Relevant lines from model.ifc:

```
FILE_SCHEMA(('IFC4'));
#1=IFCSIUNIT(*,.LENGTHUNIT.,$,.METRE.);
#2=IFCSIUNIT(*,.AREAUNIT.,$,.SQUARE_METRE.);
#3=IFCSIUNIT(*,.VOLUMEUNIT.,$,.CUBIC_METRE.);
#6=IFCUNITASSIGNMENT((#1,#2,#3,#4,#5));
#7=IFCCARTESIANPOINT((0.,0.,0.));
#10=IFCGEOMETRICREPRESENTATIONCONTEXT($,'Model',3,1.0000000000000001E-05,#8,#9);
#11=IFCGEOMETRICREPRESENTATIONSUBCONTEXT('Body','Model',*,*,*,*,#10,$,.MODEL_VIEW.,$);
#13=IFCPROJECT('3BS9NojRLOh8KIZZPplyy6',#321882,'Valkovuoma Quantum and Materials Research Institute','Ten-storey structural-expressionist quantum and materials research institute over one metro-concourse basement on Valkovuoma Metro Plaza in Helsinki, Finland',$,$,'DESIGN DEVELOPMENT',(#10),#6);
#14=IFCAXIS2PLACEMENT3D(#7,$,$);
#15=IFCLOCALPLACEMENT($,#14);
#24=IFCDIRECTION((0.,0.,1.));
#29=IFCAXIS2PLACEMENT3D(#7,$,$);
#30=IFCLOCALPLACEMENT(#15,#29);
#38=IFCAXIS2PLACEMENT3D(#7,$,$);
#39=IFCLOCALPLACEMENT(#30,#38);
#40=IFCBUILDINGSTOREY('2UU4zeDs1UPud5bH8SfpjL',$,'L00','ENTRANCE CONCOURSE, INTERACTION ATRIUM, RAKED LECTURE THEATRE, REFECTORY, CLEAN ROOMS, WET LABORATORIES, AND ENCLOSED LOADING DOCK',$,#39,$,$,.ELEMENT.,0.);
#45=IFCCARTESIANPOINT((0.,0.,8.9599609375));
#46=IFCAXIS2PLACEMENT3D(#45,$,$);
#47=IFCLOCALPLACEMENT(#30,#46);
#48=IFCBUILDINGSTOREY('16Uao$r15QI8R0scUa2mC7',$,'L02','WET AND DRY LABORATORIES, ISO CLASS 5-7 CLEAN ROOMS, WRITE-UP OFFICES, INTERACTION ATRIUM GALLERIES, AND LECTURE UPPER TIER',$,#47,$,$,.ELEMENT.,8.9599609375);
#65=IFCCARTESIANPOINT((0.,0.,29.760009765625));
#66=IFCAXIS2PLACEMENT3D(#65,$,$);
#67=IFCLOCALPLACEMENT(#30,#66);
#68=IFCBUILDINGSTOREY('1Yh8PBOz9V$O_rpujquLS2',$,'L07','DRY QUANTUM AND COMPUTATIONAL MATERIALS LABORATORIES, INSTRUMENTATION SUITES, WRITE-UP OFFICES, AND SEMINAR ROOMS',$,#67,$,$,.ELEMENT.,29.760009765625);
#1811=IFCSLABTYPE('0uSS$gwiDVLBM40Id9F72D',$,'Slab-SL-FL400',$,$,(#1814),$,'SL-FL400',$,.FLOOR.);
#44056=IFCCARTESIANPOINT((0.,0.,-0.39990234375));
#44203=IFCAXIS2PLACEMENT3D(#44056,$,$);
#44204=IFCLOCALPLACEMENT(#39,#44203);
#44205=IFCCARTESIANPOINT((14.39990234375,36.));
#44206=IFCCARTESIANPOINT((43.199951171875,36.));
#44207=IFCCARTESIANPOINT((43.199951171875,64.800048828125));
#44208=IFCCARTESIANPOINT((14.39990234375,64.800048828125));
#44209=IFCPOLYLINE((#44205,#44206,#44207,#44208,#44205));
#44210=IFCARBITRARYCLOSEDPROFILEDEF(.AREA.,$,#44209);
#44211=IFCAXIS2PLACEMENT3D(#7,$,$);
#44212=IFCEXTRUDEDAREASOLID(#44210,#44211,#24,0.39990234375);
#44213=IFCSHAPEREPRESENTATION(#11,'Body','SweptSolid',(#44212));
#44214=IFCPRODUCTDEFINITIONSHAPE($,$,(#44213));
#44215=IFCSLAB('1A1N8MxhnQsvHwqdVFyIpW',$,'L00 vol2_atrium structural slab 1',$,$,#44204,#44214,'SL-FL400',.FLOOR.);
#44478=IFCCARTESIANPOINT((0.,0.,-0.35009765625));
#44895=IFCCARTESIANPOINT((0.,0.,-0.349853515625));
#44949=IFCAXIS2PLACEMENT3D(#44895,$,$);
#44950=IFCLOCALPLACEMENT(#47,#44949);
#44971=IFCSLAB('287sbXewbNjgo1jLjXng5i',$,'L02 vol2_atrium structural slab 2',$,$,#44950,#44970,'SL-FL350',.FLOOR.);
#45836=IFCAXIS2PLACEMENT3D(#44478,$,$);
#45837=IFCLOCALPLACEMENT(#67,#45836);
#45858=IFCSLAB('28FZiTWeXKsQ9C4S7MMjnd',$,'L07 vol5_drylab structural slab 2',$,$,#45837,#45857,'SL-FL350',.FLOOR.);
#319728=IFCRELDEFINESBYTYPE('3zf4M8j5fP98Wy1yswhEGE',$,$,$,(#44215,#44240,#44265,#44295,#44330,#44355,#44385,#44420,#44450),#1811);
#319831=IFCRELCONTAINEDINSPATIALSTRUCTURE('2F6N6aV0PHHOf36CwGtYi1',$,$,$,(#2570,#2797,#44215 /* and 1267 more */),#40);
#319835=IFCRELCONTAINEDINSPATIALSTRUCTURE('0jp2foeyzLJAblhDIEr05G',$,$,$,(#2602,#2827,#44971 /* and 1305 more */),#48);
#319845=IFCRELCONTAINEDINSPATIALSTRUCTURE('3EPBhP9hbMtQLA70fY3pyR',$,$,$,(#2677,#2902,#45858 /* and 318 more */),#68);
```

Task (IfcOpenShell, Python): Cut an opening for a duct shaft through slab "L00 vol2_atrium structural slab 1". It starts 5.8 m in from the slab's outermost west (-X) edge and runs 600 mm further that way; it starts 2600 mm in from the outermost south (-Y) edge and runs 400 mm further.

```python
import numpy as np
import ifcopenshell
import ifcopenshell.api.feature
import ifcopenshell.api.geometry
import ifcopenshell.api.root
import ifcopenshell.geom
import ifcopenshell.util.placement
import ifcopenshell.util.representation
import ifcopenshell.util.shape
import ifcopenshell.util.unit

model = ifcopenshell.open("model.ifc")
unit_scale = ifcopenshell.util.unit.calculate_unit_scale(model)
settings = ifcopenshell.geom.settings()


def volume(element):
    """Net volume in cubic metres, openings subtracted."""
    shape = ifcopenshell.geom.create_shape(settings, element)
    return ifcopenshell.util.shape.get_volume(shape.geometry)


slab = model.by_guid("1A1N8MxhnQsvHwqdVFyIpW")
before = volume(slab)

# Extent in the slab's own axes, in metres. The edges named are its -X and -Y sides.
slab_shape = ifcopenshell.geom.create_shape(settings, slab)
vertices = ifcopenshell.util.shape.get_vertices(slab_shape.geometry)
x_min, y_min, bottom = vertices.min(axis=0)
top = vertices[:, 2].max()

opening = ifcopenshell.api.root.create_entity(model, ifc_class="IfcOpeningElement", name="Duct shaft opening", predefined_type="OPENING")
context = ifcopenshell.util.representation.get_context(model, "Model", "Body", "MODEL_VIEW")
width, depth = 0.6, 0.4
outline = [(0.0, 0.0), (width, 0.0), (width, depth), (0.0, depth), (0.0, 0.0)]
# Overshoot both faces by 50 mm so the cut is clean.
shape = ifcopenshell.api.geometry.add_slab_representation(
    model, context=context, depth=top - bottom + 0.1, polyline=outline
)
ifcopenshell.api.geometry.assign_representation(model, product=opening, representation=shape)

matrix = ifcopenshell.util.placement.get_local_placement(slab.ObjectPlacement)
matrix[:, 3] = matrix @ np.append(np.array([x_min + 5.8, y_min + 2.6, bottom - 0.05]) / unit_scale, 1.0)
ifcopenshell.api.geometry.edit_object_placement(model, product=opening, matrix=matrix, is_si=False)
ifcopenshell.api.feature.add_feature(model, feature=opening, element=slab)

after = volume(slab)

print(f"slab volume {before:.3f} -> {after:.3f} m3")

model.write("model_rev.ifc")
```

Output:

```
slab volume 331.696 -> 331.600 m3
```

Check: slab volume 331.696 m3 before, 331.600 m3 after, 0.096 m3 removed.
